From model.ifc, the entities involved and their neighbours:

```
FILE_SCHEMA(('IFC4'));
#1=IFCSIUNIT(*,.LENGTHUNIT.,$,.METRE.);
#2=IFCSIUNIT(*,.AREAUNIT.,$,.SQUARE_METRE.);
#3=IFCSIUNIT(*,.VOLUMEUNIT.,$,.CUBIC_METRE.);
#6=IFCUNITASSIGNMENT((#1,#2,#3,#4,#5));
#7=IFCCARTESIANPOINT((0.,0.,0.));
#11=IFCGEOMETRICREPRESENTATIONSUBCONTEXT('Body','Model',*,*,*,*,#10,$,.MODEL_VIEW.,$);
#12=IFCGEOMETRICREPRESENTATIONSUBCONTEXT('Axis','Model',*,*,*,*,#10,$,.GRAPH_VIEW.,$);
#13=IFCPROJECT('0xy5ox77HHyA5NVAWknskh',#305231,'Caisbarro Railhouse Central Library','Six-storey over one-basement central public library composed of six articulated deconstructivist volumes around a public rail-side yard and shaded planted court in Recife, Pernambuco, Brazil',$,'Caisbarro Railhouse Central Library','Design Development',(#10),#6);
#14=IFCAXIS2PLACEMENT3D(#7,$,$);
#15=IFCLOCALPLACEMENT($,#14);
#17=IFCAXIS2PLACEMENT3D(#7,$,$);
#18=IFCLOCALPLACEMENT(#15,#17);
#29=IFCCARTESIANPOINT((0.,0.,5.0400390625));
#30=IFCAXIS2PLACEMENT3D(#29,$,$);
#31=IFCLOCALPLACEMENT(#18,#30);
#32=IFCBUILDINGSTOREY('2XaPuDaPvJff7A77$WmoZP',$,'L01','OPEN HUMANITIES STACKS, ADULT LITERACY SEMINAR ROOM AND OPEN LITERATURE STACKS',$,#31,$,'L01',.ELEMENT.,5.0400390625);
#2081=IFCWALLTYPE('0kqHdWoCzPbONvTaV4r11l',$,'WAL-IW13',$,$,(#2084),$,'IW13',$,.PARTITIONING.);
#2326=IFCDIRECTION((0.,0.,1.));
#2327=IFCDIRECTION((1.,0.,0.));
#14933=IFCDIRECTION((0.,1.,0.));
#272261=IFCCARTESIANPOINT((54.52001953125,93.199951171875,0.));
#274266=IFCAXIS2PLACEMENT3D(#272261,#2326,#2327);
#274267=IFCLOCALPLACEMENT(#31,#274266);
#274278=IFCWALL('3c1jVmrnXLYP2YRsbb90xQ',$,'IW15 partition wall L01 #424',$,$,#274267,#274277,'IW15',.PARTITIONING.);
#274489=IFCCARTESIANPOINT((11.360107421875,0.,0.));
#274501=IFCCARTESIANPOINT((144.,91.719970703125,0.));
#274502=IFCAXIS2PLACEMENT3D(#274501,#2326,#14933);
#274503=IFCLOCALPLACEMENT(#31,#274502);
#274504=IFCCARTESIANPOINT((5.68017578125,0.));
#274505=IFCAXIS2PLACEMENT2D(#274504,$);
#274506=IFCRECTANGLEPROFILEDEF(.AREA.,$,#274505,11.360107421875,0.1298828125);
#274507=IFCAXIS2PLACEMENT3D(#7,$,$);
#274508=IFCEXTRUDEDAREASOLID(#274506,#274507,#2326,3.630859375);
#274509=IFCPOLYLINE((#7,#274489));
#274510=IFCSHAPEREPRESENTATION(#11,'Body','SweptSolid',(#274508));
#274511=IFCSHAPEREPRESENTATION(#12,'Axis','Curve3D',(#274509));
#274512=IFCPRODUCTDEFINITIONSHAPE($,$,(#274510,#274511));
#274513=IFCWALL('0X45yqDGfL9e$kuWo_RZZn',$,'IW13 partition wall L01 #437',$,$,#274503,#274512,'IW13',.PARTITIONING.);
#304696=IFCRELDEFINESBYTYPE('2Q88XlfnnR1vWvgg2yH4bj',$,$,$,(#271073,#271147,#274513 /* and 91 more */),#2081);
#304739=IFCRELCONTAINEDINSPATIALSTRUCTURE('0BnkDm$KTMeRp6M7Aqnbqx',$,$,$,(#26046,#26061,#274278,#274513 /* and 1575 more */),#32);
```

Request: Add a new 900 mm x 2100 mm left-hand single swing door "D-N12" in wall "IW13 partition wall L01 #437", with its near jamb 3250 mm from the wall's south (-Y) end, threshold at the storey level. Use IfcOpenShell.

```python
import numpy as np
import ifcopenshell
import ifcopenshell.api.feature
import ifcopenshell.api.geometry
import ifcopenshell.api.root
import ifcopenshell.api.spatial
import ifcopenshell.geom
import ifcopenshell.util.element
import ifcopenshell.util.placement
import ifcopenshell.util.representation
import ifcopenshell.util.shape
import ifcopenshell.util.unit

model = ifcopenshell.open("model.ifc")
unit_scale = ifcopenshell.util.unit.calculate_unit_scale(model)
settings = ifcopenshell.geom.settings()


def volume(element):
    """Net volume in cubic metres, openings subtracted."""
    shape = ifcopenshell.geom.create_shape(settings, element)
    return ifcopenshell.util.shape.get_volume(shape.geometry)


wall = model.by_guid("0X45yqDGfL9e$kuWo_RZZn")
storey = ifcopenshell.util.element.get_container(wall, ifc_class="IfcBuildingStorey")
context = ifcopenshell.util.representation.get_context(model, "Model", "Body", "MODEL_VIEW")
before = volume(wall)

width, height, from_end, sill = 0.9, 2.1, 3.25, 0.0  # metres

# The wall runs along its own X axis, and the end named is its -X end.
wall_shape = ifcopenshell.geom.create_shape(settings, wall)
x, y, z = ifcopenshell.util.shape.get_vertices(wall_shape.geometry).T
start = x.min() + from_end
face, thickness = float(y.min()), float(y.max() - y.min())
wall_matrix = ifcopenshell.util.placement.get_local_placement(wall.ObjectPlacement)
level = ifcopenshell.util.placement.get_local_placement(storey.ObjectPlacement)[2, 3]


def in_wall(x, y):
    """Placement at x, y metres in the wall's axes, at sill height."""
    matrix = wall_matrix.copy()
    matrix[:, 3] = wall_matrix @ np.array([x / unit_scale, y / unit_scale, 0.0, 1.0])
    matrix[2, 3] = level + sill / unit_scale
    return matrix


# Opening: a box that overshoots both wall faces by 50 mm.
opening = ifcopenshell.api.root.create_entity(model, ifc_class="IfcOpeningElement", predefined_type="OPENING")
box = ifcopenshell.api.geometry.add_wall_representation(
    model, context=context, length=width, height=height, thickness=thickness + 0.1
)
ifcopenshell.api.geometry.assign_representation(model, product=opening, representation=box)
ifcopenshell.api.geometry.edit_object_placement(model, product=opening, matrix=in_wall(start, face - 0.05), is_si=False)
ifcopenshell.api.feature.add_feature(model, feature=opening, element=wall)

door = ifcopenshell.api.root.create_entity(model, ifc_class="IfcDoor", name="D-N12", predefined_type="DOOR")
door.OverallWidth, door.OverallHeight = width / unit_scale, height / unit_scale
door.OperationType = "SINGLE_SWING_LEFT"
body = ifcopenshell.api.geometry.add_door_representation(
    model,
    context=context,
    overall_width=door.OverallWidth,
    overall_height=door.OverallHeight,
    operation_type="SINGLE_SWING_LEFT",
    lining_properties={"LiningDepth": thickness / unit_scale, "ThresholdDepth": thickness / unit_scale},
)
ifcopenshell.api.geometry.assign_representation(model, product=door, representation=body)
ifcopenshell.api.spatial.assign_container(model, products=[door], relating_structure=storey)
ifcopenshell.api.feature.add_filling(model, opening=opening, element=door)

# The lining spans the wall, so the door starts at the wall face.
ifcopenshell.api.geometry.edit_object_placement(model, product=door, matrix=in_wall(start, face), is_si=False)

after = volume(wall)

print(f"wall volume {before:.3f} -> {after:.3f} m3")

model.write("model_rev.ifc")
```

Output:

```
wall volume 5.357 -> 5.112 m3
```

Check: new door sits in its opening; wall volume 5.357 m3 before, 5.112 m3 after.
